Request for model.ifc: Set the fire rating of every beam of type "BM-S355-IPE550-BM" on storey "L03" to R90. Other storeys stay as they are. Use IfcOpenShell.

First a look at what the model holds.

```python
import ifcopenshell
import ifcopenshell.util.element

model = ifcopenshell.open("model.ifc")
print(model.schema)
storey = next(s for s in model.by_type("IfcBuildingStorey") if s.Name == "L03")
beams = [e for e in ifcopenshell.util.element.get_decomposition(storey) if e.is_a("IfcBeam")]
seen = {}
for e in beams:
    element_type = ifcopenshell.util.element.get_type(e)
    key = (element_type.Name if element_type != e and element_type else None, ifcopenshell.util.element.get_pset(e, "Pset_BeamCommon", "FireRating"))
    seen[key] = seen.get(key, 0) + 1
for (name, value), count in sorted(seen.items(), key=str):
    print(count, "x", name, "|", value)
```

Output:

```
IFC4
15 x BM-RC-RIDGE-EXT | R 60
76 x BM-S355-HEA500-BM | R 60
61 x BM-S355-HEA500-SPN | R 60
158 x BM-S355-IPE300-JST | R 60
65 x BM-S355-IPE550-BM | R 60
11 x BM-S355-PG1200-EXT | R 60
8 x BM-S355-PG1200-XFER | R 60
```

```python
import ifcopenshell
import ifcopenshell.api.pset
import ifcopenshell.util.element

model = ifcopenshell.open("model.ifc")

storey = next(s for s in model.by_type("IfcBuildingStorey") if s.Name == "L03")
beams = [e for e in ifcopenshell.util.element.get_decomposition(storey) if e.is_a("IfcBeam")]

count = 0
for e in beams:
    element_type = ifcopenshell.util.element.get_type(e)
    if element_type in (None, e) or element_type.Name != "BM-S355-IPE550-BM":
        continue
    # add_pset returns the element's existing set when there is one.
    pset = ifcopenshell.api.pset.add_pset(model, product=e, name="Pset_BeamCommon")
    ifcopenshell.api.pset.edit_pset(model, pset=pset, properties={"FireRating": "R90"})
    count += 1

print(count, "beams updated")

model.write("model_v2.ifc")
```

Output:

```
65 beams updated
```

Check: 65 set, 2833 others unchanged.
